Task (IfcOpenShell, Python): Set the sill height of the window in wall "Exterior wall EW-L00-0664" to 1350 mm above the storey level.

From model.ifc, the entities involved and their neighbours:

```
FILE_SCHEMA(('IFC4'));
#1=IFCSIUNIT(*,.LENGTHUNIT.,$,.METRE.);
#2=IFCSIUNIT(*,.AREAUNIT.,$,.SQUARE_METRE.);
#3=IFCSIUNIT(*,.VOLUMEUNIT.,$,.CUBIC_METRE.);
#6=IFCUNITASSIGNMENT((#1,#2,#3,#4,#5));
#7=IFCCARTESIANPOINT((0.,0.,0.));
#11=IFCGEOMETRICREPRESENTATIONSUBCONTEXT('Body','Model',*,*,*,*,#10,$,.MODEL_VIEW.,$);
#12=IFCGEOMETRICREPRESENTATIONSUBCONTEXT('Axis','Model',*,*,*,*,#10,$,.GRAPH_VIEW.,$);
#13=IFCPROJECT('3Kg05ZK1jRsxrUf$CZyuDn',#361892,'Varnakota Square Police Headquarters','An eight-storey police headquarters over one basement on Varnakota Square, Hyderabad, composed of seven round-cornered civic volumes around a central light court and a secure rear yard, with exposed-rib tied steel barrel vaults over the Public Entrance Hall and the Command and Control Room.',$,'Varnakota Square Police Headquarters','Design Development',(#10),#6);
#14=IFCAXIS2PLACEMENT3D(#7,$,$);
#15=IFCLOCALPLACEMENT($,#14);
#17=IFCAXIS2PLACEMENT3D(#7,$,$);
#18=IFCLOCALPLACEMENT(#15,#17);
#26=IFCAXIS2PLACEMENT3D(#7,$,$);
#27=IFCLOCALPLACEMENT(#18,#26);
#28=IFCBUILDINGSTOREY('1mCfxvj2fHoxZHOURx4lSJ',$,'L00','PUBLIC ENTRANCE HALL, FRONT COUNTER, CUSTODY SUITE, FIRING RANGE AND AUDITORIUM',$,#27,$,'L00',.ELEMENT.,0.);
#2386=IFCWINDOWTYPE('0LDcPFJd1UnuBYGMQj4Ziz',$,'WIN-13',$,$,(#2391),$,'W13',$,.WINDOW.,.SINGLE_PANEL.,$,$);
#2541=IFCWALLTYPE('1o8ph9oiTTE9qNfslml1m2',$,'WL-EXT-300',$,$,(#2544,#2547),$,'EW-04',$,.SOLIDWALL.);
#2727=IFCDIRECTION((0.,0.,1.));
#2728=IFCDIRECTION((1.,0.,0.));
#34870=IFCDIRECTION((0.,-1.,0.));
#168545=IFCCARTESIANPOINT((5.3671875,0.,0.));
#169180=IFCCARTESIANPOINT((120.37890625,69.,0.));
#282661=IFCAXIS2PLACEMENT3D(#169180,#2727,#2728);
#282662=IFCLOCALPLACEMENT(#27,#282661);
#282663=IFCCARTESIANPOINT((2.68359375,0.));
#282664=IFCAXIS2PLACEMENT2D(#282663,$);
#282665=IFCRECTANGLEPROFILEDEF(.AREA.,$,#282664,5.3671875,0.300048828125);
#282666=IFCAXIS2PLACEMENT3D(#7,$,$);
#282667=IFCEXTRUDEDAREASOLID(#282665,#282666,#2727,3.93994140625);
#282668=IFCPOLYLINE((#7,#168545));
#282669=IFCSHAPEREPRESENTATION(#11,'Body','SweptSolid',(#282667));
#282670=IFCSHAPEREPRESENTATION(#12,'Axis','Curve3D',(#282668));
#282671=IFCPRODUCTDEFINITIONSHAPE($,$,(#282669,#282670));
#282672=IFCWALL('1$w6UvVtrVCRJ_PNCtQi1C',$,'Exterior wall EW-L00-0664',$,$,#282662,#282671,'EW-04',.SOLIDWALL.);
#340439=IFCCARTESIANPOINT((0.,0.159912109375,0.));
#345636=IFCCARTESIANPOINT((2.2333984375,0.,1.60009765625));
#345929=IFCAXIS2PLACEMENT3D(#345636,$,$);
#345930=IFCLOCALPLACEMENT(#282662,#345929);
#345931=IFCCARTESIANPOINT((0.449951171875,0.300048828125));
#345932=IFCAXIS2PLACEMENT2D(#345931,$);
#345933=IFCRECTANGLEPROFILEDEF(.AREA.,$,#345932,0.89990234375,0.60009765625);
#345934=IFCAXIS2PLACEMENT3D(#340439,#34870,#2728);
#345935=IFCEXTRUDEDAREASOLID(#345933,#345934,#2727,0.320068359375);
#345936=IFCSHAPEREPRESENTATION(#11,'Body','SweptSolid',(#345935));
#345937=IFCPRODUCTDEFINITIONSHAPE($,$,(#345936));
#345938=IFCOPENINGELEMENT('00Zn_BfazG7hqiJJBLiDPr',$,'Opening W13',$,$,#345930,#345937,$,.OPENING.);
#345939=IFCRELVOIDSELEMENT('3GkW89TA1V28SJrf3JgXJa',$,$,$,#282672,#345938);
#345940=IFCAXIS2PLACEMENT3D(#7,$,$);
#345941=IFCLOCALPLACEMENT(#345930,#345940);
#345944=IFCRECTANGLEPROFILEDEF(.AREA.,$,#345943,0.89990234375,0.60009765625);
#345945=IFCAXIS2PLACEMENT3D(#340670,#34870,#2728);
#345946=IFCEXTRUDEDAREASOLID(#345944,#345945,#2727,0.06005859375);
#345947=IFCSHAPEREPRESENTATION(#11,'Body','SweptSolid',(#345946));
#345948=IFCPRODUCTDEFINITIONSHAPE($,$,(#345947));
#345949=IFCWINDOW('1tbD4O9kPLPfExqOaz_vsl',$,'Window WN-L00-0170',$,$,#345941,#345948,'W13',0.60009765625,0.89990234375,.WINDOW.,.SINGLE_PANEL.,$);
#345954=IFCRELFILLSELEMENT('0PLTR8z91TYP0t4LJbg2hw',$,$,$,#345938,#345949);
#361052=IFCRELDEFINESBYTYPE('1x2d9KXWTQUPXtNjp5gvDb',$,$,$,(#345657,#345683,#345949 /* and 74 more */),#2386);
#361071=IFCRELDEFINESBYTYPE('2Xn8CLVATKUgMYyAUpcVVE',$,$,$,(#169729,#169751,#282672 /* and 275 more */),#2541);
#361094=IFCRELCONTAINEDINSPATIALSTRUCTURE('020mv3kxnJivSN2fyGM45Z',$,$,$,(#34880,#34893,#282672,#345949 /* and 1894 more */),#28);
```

```python
import numpy as np
import ifcopenshell
import ifcopenshell.api.geometry
import ifcopenshell.geom
import ifcopenshell.util.element
import ifcopenshell.util.placement
import ifcopenshell.util.shape
import ifcopenshell.util.unit

model = ifcopenshell.open("model.ifc")
unit_scale = ifcopenshell.util.unit.calculate_unit_scale(model)

window = model.by_id(345949)
opening = window.FillsVoids[0].RelatingOpeningElement
storey = ifcopenshell.util.element.get_container(window, ifc_class="IfcBuildingStorey")
level = ifcopenshell.util.placement.get_local_placement(storey.ObjectPlacement)[2, 3]

# The opening's origin need not be at the sill, so measure its lowest point.
shape = ifcopenshell.geom.create_shape(ifcopenshell.geom.settings(), opening)
bottom = ifcopenshell.util.shape.get_shape_bottom_elevation(shape, shape.geometry) / unit_scale
dz = level + 1.35 - bottom

shift = np.array([0.0, 0.0, dz])
# The window is placed relative to its opening, so it follows when the opening moves.
matrix = ifcopenshell.util.placement.get_local_placement(opening.ObjectPlacement)
matrix[:3, 3] += shift
ifcopenshell.api.geometry.edit_object_placement(
    model, product=opening, matrix=matrix, is_si=False, should_transform_children=True
)

print(f"moved by {dz * unit_scale:+.3f} m")

model.write("model_rev.ifc")
```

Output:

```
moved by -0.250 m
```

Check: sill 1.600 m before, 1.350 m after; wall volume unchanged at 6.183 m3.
